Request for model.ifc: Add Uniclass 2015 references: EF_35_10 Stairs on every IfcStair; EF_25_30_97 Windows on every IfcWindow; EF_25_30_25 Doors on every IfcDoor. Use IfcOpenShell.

First a look at what the model holds.

```python
import ifcopenshell

model = ifcopenshell.open("model.ifc")
print(model.schema)
print("classifications:", [c.Name for c in model.by_type("IfcClassification")])
for ifc_class in ("IfcDoor", "IfcRoof", "IfcStair", "IfcWall", "IfcWindow"):
    print(ifc_class, len(model.by_type(ifc_class)))
```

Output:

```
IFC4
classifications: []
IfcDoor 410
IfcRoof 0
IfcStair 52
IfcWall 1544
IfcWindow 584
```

```python
import ifcopenshell
import ifcopenshell.api.classification

model = ifcopenshell.open("model.ifc")

system = ifcopenshell.api.classification.add_classification(model, classification="Uniclass 2015")

codes = {
    "IfcStair": ("EF_35_10", "Stairs"),
    "IfcWindow": ("EF_25_30_97", "Windows"),
    "IfcDoor": ("EF_25_30_25", "Doors"),
}
for ifc_class, (code, name) in codes.items():
    products = model.by_type(ifc_class)
    ifcopenshell.api.classification.add_reference(
        model, products=products, classification=system, identification=code, name=name
    )
    print(code, len(products))

model.write("model_edited.ifc")
```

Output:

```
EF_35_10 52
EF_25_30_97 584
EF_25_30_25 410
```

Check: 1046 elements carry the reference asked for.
